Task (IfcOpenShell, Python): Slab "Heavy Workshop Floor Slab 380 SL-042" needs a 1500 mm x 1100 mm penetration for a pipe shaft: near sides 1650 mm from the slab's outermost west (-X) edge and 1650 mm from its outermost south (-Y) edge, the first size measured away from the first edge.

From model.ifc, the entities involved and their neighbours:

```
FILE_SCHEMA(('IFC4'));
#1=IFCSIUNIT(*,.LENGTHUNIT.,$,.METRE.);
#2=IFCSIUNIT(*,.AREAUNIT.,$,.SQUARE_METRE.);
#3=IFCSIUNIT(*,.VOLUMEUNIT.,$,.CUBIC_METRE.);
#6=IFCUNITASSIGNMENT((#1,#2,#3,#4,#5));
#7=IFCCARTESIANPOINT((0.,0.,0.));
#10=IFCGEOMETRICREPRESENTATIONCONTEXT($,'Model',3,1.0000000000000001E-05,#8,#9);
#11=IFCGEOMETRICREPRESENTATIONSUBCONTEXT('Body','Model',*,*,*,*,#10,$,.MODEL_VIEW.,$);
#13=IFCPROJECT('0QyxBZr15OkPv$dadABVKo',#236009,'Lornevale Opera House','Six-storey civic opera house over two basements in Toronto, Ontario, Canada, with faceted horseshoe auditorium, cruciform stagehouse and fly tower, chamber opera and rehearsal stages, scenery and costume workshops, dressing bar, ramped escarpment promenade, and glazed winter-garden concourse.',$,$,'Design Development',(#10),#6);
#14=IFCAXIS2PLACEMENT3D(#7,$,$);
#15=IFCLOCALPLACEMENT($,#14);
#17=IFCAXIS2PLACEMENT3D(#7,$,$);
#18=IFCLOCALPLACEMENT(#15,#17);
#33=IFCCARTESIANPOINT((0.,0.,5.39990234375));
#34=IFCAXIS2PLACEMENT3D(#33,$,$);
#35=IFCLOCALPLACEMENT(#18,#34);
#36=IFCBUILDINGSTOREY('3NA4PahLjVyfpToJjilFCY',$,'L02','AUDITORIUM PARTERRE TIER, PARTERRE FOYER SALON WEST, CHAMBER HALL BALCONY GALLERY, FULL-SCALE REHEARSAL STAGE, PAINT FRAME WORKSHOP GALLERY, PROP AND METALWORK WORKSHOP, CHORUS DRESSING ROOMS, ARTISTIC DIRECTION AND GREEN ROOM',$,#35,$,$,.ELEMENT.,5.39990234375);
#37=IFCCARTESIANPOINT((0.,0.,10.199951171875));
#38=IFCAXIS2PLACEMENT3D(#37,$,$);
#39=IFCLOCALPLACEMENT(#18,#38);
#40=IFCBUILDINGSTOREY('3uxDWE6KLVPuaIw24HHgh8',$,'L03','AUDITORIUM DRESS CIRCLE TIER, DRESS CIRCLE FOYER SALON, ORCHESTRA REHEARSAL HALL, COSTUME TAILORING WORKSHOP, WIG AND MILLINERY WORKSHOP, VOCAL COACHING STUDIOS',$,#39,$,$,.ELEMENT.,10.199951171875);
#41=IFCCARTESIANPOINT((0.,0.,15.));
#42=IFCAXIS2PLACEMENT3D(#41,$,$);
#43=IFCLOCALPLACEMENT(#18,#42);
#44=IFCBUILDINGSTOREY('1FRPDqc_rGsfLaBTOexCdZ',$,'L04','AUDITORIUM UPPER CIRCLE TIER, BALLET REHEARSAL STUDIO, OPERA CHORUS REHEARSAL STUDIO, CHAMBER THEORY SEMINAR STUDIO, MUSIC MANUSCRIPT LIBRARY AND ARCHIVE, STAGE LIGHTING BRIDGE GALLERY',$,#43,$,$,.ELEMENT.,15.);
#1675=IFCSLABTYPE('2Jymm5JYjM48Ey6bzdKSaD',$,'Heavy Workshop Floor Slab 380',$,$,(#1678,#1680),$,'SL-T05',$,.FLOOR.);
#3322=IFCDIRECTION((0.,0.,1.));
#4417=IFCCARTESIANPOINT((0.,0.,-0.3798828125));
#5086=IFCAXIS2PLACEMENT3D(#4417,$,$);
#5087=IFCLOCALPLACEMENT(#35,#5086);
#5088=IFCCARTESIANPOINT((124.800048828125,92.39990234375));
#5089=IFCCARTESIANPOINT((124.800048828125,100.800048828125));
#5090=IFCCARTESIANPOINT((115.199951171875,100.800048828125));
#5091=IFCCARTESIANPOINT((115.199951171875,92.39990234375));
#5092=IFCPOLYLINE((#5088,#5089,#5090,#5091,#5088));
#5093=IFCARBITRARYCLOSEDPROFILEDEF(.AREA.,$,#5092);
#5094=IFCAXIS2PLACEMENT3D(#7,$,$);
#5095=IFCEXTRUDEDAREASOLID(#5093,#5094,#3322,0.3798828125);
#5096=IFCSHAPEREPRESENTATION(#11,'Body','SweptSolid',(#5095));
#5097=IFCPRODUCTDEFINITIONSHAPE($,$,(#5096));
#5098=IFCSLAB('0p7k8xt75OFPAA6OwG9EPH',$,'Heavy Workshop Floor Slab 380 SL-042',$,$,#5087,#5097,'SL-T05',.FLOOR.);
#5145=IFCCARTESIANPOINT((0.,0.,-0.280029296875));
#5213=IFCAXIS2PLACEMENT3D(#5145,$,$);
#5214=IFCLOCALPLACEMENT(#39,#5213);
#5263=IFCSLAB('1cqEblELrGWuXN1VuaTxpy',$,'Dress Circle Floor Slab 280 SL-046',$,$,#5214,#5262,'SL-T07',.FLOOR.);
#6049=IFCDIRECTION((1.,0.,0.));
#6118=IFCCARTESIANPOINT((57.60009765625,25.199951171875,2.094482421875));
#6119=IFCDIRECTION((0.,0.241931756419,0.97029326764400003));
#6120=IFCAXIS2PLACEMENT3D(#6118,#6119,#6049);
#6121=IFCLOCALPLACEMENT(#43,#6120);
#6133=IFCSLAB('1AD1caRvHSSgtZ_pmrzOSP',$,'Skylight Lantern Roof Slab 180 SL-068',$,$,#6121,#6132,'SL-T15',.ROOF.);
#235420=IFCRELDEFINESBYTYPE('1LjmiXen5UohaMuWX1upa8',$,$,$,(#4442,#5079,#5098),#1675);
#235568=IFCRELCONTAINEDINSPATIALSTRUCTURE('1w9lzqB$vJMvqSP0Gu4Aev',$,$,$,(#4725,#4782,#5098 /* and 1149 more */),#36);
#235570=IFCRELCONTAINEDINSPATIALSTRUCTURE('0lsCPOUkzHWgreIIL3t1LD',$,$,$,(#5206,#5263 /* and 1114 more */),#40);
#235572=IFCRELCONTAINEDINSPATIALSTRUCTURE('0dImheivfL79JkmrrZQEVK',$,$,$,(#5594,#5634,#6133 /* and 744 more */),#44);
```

```python
import numpy as np
import ifcopenshell
import ifcopenshell.api.feature
import ifcopenshell.api.geometry
import ifcopenshell.api.root
import ifcopenshell.geom
import ifcopenshell.util.placement
import ifcopenshell.util.representation
import ifcopenshell.util.shape
import ifcopenshell.util.unit

model = ifcopenshell.open("model.ifc")
unit_scale = ifcopenshell.util.unit.calculate_unit_scale(model)
settings = ifcopenshell.geom.settings()


def volume(element):
    """Net volume in cubic metres, openings subtracted."""
    shape = ifcopenshell.geom.create_shape(settings, element)
    return ifcopenshell.util.shape.get_volume(shape.geometry)


slab = model.by_guid("0p7k8xt75OFPAA6OwG9EPH")
before = volume(slab)

# Extent in the slab's own axes, in metres. The edges named are its -X and -Y sides.
slab_shape = ifcopenshell.geom.create_shape(settings, slab)
vertices = ifcopenshell.util.shape.get_vertices(slab_shape.geometry)
x_min, y_min, bottom = vertices.min(axis=0)
top = vertices[:, 2].max()

opening = ifcopenshell.api.root.create_entity(model, ifc_class="IfcOpeningElement", name="Pipe shaft opening", predefined_type="OPENING")
context = ifcopenshell.util.representation.get_context(model, "Model", "Body", "MODEL_VIEW")
width, depth = 1.5, 1.1
outline = [(0.0, 0.0), (width, 0.0), (width, depth), (0.0, depth), (0.0, 0.0)]
# Overshoot both faces by 50 mm so the cut is clean.
shape = ifcopenshell.api.geometry.add_slab_representation(
    model, context=context, depth=top - bottom + 0.1, polyline=outline
)
ifcopenshell.api.geometry.assign_representation(model, product=opening, representation=shape)

matrix = ifcopenshell.util.placement.get_local_placement(slab.ObjectPlacement)
matrix[:, 3] = matrix @ np.append(np.array([x_min + 1.65, y_min + 1.65, bottom - 0.05]) / unit_scale, 1.0)
ifcopenshell.api.geometry.edit_object_placement(model, product=opening, matrix=matrix, is_si=False)
ifcopenshell.api.feature.add_feature(model, feature=opening, element=slab)

after = volume(slab)

print(f"slab volume {before:.3f} -> {after:.3f} m3")

model.write("model_updated.ifc")
```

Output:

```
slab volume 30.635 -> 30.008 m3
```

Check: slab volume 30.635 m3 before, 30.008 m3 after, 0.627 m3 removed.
